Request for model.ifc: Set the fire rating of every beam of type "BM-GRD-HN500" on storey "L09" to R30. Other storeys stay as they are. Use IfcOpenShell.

First a look at what the model holds.

```python
import ifcopenshell
import ifcopenshell.util.element

model = ifcopenshell.open("model.ifc")
print(model.schema)
storey = next(s for s in model.by_type("IfcBuildingStorey") if s.Name == "L09")
beams = [e for e in ifcopenshell.util.element.get_decomposition(storey) if e.is_a("IfcBeam")]
seen = {}
for e in beams:
    element_type = ifcopenshell.util.element.get_type(e)
    key = (element_type.Name if element_type != e and element_type else None, ifcopenshell.util.element.get_pset(e, "Pset_BeamCommon", "FireRating"))
    seen[key] = seen.get(key, 0) + 1
for (name, value), count in sorted(seen.items(), key=str):
    print(count, "x", name, "|", value)
```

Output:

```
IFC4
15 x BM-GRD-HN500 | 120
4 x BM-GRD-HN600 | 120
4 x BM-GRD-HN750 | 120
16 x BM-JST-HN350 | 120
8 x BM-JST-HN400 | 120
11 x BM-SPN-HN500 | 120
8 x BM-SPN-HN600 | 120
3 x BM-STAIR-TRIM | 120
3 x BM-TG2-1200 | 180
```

```python
import ifcopenshell
import ifcopenshell.api.pset
import ifcopenshell.util.element

model = ifcopenshell.open("model.ifc")

storey = next(s for s in model.by_type("IfcBuildingStorey") if s.Name == "L09")
beams = [e for e in ifcopenshell.util.element.get_decomposition(storey) if e.is_a("IfcBeam")]

count = 0
for e in beams:
    element_type = ifcopenshell.util.element.get_type(e)
    if element_type in (None, e) or element_type.Name != "BM-GRD-HN500":
        continue
    # add_pset returns the element's existing set when there is one.
    pset = ifcopenshell.api.pset.add_pset(model, product=e, name="Pset_BeamCommon")
    ifcopenshell.api.pset.edit_pset(model, pset=pset, properties={"FireRating": "R30"})
    count += 1

print(count, "beams updated")

model.write("model-out.ifc")
```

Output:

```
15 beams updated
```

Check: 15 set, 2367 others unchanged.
